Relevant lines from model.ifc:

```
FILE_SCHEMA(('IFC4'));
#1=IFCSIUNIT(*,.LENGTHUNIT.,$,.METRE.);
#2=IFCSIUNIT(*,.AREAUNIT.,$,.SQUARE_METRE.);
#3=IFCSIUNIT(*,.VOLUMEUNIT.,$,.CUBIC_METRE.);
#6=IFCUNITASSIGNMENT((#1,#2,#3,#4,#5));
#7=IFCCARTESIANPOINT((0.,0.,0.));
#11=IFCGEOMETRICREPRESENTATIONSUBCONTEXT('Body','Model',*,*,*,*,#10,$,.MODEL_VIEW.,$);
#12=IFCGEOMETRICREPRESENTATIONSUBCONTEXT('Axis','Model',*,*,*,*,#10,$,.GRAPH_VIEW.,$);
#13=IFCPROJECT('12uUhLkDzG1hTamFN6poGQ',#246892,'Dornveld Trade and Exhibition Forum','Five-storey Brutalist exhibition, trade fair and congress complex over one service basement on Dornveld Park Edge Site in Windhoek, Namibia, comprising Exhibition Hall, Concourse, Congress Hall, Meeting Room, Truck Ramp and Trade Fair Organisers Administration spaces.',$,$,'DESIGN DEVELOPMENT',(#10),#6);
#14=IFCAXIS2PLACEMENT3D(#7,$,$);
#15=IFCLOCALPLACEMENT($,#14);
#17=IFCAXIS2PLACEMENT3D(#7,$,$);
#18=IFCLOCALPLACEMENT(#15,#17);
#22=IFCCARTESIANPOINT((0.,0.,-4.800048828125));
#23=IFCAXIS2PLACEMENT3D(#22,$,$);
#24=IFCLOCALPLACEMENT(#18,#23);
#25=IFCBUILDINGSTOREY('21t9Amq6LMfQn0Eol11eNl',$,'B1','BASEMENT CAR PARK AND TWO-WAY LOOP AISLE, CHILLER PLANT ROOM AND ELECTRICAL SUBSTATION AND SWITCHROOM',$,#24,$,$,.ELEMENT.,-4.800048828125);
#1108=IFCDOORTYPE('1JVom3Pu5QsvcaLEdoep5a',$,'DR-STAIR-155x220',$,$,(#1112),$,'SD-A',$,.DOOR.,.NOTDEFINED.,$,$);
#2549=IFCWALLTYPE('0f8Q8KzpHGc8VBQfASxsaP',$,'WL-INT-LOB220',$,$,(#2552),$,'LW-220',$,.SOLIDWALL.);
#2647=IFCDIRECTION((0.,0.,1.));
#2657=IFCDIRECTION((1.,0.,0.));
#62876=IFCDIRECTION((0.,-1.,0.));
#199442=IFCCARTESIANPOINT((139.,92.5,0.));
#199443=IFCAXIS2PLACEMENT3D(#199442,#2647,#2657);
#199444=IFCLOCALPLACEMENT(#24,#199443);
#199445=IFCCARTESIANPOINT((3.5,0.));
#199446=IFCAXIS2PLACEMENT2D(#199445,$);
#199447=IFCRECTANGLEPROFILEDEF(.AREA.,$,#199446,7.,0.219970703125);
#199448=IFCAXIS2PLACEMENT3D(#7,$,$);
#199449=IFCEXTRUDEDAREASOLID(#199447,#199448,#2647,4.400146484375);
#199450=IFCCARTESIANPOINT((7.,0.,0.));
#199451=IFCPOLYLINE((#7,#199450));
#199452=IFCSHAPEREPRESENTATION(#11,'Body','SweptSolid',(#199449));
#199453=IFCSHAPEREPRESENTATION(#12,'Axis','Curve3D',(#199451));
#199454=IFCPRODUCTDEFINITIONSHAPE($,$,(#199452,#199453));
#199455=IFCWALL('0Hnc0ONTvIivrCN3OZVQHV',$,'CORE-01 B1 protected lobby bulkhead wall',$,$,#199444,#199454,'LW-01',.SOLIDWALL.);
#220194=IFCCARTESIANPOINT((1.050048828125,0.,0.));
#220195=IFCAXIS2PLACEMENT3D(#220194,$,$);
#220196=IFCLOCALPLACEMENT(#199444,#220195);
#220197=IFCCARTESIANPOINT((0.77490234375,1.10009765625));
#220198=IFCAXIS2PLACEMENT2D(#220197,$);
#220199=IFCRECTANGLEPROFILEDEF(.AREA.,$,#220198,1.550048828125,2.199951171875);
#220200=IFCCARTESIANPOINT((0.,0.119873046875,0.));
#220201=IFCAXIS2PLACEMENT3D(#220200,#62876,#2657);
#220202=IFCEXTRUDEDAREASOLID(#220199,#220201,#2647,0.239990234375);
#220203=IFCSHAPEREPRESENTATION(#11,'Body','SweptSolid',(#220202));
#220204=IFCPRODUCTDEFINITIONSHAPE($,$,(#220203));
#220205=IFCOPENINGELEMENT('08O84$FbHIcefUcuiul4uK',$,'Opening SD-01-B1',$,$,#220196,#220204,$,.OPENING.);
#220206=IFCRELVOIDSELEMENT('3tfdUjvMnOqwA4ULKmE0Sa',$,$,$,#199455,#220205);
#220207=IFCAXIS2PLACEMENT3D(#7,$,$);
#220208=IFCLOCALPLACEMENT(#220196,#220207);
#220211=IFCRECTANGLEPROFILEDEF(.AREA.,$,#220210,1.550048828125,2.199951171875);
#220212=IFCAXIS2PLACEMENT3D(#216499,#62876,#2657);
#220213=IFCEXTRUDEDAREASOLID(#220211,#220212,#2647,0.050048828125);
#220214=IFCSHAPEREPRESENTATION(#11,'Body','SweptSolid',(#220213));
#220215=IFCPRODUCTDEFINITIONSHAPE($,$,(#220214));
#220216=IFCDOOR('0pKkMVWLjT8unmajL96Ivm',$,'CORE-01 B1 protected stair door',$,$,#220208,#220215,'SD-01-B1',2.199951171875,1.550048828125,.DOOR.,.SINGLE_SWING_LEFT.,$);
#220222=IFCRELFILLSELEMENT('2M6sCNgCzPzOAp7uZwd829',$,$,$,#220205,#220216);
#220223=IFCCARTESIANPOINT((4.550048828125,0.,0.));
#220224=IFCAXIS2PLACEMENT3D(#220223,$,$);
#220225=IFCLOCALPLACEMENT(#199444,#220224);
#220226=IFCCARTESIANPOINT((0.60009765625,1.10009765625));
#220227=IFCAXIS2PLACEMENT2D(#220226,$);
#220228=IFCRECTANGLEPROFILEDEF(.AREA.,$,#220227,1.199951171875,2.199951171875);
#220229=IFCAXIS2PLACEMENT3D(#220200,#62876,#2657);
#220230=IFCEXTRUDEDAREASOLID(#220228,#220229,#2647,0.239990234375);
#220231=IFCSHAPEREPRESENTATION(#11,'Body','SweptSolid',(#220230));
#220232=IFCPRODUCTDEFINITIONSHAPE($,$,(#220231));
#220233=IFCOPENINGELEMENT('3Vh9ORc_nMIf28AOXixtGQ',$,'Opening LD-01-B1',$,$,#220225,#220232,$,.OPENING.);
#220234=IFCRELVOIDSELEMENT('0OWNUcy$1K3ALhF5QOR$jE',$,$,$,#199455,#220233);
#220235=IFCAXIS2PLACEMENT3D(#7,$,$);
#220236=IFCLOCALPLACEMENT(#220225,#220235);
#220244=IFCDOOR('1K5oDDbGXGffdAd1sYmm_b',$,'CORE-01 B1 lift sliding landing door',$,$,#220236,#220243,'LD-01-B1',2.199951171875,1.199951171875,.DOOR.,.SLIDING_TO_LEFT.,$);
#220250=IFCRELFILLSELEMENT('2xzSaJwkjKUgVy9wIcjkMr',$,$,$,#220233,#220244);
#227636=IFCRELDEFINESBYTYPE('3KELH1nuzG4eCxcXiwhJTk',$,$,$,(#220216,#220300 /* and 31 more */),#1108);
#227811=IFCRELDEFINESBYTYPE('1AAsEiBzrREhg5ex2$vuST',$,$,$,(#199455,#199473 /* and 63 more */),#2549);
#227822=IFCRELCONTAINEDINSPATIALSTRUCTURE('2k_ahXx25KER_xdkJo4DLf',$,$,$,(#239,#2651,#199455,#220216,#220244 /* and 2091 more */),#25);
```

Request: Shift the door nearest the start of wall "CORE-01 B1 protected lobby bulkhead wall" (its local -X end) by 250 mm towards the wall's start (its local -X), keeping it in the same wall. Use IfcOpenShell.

```python
import ifcopenshell
import ifcopenshell.api.geometry
import ifcopenshell.util.placement
import ifcopenshell.util.unit

model = ifcopenshell.open("model.ifc")
unit_scale = ifcopenshell.util.unit.calculate_unit_scale(model)

door = model.by_guid("0pKkMVWLjT8unmajL96Ivm")
opening = door.FillsVoids[0].RelatingOpeningElement
wall = opening.VoidsElements[0].RelatingBuildingElement

wall_matrix = ifcopenshell.util.placement.get_local_placement(wall.ObjectPlacement)
shift = wall_matrix[:3, 0] * -0.25 / unit_scale
before = ifcopenshell.util.placement.get_local_placement(door.ObjectPlacement)[:3, 3].copy()

# The door is placed relative to its opening, so it follows when the opening moves.
matrix = ifcopenshell.util.placement.get_local_placement(opening.ObjectPlacement)
matrix[:3, 3] += shift
ifcopenshell.api.geometry.edit_object_placement(
    model, product=opening, matrix=matrix, is_si=False, should_transform_children=True
)

after = ifcopenshell.util.placement.get_local_placement(door.ObjectPlacement)[:3, 3]
print("door moved by", (after - before).round(3) + 0.0)

model.write("model-out.ifc")
```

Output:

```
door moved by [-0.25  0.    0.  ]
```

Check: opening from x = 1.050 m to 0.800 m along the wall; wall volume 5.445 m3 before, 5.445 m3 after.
